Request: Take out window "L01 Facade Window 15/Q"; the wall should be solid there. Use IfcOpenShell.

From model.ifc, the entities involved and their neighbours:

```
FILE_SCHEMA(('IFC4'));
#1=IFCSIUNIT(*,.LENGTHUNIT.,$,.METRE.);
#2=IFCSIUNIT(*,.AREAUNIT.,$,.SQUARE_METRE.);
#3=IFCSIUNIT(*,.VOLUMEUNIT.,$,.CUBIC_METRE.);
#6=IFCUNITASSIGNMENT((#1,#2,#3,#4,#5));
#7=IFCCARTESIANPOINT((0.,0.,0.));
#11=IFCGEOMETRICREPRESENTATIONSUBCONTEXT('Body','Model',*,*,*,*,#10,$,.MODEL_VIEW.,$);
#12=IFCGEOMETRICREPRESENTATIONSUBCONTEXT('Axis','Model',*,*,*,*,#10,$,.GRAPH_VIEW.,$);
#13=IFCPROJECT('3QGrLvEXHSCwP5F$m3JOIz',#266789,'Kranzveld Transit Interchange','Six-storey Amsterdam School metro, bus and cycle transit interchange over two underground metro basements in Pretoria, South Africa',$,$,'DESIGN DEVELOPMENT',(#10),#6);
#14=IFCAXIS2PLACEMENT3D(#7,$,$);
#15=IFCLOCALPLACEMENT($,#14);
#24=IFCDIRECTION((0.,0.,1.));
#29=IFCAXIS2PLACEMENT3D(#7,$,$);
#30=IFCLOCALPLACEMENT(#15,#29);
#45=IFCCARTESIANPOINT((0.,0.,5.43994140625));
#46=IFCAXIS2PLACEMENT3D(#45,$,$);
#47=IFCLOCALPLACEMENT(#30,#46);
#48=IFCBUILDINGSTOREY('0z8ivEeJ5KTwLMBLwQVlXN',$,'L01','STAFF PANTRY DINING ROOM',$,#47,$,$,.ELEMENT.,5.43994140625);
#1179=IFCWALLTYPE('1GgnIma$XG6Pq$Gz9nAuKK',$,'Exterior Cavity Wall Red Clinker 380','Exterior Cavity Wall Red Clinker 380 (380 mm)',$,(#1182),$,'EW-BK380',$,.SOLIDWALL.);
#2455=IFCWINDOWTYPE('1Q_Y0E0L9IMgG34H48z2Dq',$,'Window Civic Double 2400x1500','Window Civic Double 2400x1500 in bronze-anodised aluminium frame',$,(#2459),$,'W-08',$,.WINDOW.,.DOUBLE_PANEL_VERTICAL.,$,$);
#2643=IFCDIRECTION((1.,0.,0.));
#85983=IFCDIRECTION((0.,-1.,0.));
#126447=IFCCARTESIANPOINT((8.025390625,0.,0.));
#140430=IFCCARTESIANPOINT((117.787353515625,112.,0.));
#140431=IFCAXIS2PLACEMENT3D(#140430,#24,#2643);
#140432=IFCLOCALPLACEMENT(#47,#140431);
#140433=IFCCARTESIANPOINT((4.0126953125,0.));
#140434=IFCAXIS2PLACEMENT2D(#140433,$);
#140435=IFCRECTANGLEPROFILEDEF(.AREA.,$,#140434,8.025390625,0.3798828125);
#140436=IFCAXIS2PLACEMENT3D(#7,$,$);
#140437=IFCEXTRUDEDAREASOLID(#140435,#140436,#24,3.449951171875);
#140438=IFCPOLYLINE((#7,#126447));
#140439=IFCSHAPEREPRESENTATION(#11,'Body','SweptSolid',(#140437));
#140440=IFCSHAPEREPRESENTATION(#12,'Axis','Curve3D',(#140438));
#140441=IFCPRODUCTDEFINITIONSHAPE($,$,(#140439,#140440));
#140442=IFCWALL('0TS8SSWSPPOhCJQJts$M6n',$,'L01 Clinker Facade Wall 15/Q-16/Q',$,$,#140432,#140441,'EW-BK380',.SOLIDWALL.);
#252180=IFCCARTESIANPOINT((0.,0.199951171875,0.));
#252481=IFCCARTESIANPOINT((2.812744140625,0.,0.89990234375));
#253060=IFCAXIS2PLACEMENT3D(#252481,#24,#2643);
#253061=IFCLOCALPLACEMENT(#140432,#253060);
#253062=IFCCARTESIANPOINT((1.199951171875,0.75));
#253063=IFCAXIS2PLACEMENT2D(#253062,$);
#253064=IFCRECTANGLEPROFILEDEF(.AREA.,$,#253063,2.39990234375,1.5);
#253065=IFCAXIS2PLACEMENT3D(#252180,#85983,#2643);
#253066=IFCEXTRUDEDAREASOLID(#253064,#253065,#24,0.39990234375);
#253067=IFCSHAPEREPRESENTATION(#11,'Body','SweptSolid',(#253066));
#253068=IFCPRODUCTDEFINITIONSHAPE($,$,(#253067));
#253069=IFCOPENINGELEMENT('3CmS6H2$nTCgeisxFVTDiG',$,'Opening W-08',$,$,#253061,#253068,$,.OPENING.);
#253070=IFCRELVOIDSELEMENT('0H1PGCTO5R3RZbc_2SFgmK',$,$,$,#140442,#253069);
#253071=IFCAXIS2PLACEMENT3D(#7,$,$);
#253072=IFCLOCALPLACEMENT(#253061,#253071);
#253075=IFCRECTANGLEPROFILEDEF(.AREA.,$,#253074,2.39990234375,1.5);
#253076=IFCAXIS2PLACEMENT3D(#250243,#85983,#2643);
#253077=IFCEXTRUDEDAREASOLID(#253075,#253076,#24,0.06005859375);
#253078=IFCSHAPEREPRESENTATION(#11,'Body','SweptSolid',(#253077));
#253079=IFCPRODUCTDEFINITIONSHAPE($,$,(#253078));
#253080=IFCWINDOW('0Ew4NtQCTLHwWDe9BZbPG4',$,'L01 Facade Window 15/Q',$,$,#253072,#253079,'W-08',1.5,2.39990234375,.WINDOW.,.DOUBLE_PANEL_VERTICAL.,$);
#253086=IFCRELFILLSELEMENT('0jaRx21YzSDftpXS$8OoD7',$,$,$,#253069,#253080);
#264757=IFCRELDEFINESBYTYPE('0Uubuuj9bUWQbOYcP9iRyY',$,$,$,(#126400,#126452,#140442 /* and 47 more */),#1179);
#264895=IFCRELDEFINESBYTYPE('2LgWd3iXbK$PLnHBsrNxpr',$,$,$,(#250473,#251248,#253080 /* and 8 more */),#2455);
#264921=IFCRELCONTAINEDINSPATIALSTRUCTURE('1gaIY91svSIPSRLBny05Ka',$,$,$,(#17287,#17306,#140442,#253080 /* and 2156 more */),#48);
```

```python
import ifcopenshell
import ifcopenshell.api.feature
import ifcopenshell.api.root
import ifcopenshell.geom
import ifcopenshell.util.shape

model = ifcopenshell.open("model.ifc")
settings = ifcopenshell.geom.settings()


def volume(element):
    """Net volume in cubic metres, openings subtracted."""
    shape = ifcopenshell.geom.create_shape(settings, element)
    return ifcopenshell.util.shape.get_volume(shape.geometry)


window = model.by_guid("0Ew4NtQCTLHwWDe9BZbPG4")
opening = window.FillsVoids[0].RelatingOpeningElement
wall = opening.VoidsElements[0].RelatingBuildingElement
before = volume(wall)

ifcopenshell.api.root.remove_product(model, product=window)
ifcopenshell.api.feature.remove_feature(model, feature=opening)

after = volume(wall)

print(f"wall volume {before:.3f} -> {after:.3f} m3")

model.write("model_edited.ifc")
```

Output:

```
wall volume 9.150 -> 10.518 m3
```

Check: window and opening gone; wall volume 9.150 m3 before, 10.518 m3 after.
